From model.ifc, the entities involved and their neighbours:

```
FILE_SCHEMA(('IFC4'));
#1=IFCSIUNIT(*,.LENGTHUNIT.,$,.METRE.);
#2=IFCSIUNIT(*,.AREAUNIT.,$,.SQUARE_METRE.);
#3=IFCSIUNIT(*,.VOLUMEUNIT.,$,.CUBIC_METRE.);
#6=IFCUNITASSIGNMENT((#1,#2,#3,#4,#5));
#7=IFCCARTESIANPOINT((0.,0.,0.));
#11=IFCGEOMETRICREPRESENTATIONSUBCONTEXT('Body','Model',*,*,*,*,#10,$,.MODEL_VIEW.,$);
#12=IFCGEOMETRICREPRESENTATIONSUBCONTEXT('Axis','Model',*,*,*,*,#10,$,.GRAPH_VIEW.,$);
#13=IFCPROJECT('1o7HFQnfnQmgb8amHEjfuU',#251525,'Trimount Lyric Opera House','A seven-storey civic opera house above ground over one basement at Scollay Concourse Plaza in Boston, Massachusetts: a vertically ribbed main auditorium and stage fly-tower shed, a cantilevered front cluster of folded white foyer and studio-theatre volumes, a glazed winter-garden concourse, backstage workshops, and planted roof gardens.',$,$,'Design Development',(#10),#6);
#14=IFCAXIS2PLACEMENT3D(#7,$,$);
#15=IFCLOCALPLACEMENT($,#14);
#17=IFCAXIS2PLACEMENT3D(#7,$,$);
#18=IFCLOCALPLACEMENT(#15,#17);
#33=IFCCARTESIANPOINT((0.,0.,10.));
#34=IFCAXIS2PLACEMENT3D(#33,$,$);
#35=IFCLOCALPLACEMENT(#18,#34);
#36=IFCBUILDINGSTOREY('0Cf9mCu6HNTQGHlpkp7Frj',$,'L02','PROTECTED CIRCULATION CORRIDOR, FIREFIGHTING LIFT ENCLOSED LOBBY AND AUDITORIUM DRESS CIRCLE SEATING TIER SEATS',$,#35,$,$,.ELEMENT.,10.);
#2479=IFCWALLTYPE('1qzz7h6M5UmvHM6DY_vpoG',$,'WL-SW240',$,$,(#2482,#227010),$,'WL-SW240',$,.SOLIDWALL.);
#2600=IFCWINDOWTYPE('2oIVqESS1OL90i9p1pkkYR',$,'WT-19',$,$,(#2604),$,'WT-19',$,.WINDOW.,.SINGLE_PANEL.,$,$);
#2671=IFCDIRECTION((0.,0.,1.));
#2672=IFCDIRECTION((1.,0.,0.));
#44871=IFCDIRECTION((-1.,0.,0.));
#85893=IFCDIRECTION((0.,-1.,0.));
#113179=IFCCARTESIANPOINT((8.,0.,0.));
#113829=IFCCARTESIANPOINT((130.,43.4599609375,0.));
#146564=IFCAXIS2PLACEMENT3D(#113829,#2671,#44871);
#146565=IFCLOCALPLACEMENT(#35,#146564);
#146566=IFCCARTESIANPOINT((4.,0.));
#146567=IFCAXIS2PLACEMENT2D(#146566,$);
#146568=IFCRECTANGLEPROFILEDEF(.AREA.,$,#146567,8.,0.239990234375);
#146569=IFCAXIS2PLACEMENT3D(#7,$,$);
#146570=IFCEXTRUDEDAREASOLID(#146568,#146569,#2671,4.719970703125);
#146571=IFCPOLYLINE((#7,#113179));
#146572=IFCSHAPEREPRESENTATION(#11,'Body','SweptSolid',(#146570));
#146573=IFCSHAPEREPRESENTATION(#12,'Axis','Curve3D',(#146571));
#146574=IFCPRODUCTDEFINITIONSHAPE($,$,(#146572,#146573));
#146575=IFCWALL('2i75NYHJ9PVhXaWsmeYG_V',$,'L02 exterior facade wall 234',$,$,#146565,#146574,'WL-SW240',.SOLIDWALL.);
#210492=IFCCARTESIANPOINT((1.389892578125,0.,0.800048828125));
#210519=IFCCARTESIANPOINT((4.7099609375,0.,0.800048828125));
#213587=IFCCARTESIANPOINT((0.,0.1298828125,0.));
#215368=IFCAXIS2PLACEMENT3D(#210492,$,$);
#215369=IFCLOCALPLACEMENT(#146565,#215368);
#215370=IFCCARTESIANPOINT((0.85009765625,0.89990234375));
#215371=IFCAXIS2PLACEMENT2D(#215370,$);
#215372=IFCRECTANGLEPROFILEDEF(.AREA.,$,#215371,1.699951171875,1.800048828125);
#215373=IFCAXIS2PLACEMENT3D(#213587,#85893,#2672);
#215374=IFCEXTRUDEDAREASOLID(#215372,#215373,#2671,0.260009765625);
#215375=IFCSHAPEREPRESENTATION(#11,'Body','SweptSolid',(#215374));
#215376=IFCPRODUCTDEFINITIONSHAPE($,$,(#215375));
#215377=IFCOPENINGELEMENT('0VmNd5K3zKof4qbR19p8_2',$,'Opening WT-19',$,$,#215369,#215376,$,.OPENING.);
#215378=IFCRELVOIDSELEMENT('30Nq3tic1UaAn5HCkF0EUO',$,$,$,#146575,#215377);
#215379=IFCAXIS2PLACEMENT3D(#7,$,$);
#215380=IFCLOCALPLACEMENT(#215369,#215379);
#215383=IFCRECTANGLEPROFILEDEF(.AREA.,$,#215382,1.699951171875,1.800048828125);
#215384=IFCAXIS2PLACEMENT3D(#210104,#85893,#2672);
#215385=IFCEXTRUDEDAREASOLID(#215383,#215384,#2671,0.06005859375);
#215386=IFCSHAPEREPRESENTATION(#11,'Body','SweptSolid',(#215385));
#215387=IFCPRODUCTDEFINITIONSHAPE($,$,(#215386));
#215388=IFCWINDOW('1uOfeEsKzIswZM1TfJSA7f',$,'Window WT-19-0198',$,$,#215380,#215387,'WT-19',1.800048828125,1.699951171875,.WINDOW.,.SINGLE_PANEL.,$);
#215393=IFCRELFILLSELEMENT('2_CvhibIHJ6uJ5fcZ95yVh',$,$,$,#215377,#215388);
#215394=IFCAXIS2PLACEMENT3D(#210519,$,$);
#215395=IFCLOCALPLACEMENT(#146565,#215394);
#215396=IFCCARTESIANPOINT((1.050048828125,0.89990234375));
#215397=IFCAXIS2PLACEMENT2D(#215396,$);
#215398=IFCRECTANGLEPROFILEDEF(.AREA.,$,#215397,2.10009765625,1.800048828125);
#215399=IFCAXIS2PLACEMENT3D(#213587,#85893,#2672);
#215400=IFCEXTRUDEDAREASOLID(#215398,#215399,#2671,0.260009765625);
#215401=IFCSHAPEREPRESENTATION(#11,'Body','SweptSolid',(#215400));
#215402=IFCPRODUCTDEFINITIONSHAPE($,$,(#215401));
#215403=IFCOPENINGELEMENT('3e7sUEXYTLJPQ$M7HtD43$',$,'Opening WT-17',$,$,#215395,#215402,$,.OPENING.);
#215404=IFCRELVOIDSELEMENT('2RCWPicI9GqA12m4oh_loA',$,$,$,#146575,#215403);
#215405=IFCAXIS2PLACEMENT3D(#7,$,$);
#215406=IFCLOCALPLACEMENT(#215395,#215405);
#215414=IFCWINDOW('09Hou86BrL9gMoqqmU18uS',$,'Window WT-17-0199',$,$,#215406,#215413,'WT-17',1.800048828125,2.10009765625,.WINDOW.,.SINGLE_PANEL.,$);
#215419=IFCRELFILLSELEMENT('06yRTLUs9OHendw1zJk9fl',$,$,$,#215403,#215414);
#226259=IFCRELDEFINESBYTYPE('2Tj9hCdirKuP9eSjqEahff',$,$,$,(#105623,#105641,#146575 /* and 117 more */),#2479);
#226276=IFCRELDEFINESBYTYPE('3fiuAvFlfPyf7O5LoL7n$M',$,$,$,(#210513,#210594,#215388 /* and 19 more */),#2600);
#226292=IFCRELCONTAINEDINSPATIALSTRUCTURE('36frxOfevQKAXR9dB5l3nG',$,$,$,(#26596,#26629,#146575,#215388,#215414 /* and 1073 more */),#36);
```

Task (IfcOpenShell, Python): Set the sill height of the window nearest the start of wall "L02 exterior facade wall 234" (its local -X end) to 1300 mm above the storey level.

```python
import numpy as np
import ifcopenshell
import ifcopenshell.api.geometry
import ifcopenshell.geom
import ifcopenshell.util.element
import ifcopenshell.util.placement
import ifcopenshell.util.shape
import ifcopenshell.util.unit

model = ifcopenshell.open("model.ifc")
unit_scale = ifcopenshell.util.unit.calculate_unit_scale(model)

window = model.by_guid("1uOfeEsKzIswZM1TfJSA7f")
opening = window.FillsVoids[0].RelatingOpeningElement
storey = ifcopenshell.util.element.get_container(window, ifc_class="IfcBuildingStorey")
level = ifcopenshell.util.placement.get_local_placement(storey.ObjectPlacement)[2, 3]

# The opening's origin need not be at the sill, so measure its lowest point.
shape = ifcopenshell.geom.create_shape(ifcopenshell.geom.settings(), opening)
bottom = ifcopenshell.util.shape.get_shape_bottom_elevation(shape, shape.geometry) / unit_scale
dz = level + 1.3 / unit_scale - bottom

shift = np.array([0.0, 0.0, dz])
# The window is placed relative to its opening, so it follows when the opening moves.
matrix = ifcopenshell.util.placement.get_local_placement(opening.ObjectPlacement)
matrix[:3, 3] += shift
ifcopenshell.api.geometry.edit_object_placement(
    model, product=opening, matrix=matrix, is_si=False, should_transform_children=True
)

print(f"moved by {dz * unit_scale:+.3f} m")

model.write("model_v2.ifc")
```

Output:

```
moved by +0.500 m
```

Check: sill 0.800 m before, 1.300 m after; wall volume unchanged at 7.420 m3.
